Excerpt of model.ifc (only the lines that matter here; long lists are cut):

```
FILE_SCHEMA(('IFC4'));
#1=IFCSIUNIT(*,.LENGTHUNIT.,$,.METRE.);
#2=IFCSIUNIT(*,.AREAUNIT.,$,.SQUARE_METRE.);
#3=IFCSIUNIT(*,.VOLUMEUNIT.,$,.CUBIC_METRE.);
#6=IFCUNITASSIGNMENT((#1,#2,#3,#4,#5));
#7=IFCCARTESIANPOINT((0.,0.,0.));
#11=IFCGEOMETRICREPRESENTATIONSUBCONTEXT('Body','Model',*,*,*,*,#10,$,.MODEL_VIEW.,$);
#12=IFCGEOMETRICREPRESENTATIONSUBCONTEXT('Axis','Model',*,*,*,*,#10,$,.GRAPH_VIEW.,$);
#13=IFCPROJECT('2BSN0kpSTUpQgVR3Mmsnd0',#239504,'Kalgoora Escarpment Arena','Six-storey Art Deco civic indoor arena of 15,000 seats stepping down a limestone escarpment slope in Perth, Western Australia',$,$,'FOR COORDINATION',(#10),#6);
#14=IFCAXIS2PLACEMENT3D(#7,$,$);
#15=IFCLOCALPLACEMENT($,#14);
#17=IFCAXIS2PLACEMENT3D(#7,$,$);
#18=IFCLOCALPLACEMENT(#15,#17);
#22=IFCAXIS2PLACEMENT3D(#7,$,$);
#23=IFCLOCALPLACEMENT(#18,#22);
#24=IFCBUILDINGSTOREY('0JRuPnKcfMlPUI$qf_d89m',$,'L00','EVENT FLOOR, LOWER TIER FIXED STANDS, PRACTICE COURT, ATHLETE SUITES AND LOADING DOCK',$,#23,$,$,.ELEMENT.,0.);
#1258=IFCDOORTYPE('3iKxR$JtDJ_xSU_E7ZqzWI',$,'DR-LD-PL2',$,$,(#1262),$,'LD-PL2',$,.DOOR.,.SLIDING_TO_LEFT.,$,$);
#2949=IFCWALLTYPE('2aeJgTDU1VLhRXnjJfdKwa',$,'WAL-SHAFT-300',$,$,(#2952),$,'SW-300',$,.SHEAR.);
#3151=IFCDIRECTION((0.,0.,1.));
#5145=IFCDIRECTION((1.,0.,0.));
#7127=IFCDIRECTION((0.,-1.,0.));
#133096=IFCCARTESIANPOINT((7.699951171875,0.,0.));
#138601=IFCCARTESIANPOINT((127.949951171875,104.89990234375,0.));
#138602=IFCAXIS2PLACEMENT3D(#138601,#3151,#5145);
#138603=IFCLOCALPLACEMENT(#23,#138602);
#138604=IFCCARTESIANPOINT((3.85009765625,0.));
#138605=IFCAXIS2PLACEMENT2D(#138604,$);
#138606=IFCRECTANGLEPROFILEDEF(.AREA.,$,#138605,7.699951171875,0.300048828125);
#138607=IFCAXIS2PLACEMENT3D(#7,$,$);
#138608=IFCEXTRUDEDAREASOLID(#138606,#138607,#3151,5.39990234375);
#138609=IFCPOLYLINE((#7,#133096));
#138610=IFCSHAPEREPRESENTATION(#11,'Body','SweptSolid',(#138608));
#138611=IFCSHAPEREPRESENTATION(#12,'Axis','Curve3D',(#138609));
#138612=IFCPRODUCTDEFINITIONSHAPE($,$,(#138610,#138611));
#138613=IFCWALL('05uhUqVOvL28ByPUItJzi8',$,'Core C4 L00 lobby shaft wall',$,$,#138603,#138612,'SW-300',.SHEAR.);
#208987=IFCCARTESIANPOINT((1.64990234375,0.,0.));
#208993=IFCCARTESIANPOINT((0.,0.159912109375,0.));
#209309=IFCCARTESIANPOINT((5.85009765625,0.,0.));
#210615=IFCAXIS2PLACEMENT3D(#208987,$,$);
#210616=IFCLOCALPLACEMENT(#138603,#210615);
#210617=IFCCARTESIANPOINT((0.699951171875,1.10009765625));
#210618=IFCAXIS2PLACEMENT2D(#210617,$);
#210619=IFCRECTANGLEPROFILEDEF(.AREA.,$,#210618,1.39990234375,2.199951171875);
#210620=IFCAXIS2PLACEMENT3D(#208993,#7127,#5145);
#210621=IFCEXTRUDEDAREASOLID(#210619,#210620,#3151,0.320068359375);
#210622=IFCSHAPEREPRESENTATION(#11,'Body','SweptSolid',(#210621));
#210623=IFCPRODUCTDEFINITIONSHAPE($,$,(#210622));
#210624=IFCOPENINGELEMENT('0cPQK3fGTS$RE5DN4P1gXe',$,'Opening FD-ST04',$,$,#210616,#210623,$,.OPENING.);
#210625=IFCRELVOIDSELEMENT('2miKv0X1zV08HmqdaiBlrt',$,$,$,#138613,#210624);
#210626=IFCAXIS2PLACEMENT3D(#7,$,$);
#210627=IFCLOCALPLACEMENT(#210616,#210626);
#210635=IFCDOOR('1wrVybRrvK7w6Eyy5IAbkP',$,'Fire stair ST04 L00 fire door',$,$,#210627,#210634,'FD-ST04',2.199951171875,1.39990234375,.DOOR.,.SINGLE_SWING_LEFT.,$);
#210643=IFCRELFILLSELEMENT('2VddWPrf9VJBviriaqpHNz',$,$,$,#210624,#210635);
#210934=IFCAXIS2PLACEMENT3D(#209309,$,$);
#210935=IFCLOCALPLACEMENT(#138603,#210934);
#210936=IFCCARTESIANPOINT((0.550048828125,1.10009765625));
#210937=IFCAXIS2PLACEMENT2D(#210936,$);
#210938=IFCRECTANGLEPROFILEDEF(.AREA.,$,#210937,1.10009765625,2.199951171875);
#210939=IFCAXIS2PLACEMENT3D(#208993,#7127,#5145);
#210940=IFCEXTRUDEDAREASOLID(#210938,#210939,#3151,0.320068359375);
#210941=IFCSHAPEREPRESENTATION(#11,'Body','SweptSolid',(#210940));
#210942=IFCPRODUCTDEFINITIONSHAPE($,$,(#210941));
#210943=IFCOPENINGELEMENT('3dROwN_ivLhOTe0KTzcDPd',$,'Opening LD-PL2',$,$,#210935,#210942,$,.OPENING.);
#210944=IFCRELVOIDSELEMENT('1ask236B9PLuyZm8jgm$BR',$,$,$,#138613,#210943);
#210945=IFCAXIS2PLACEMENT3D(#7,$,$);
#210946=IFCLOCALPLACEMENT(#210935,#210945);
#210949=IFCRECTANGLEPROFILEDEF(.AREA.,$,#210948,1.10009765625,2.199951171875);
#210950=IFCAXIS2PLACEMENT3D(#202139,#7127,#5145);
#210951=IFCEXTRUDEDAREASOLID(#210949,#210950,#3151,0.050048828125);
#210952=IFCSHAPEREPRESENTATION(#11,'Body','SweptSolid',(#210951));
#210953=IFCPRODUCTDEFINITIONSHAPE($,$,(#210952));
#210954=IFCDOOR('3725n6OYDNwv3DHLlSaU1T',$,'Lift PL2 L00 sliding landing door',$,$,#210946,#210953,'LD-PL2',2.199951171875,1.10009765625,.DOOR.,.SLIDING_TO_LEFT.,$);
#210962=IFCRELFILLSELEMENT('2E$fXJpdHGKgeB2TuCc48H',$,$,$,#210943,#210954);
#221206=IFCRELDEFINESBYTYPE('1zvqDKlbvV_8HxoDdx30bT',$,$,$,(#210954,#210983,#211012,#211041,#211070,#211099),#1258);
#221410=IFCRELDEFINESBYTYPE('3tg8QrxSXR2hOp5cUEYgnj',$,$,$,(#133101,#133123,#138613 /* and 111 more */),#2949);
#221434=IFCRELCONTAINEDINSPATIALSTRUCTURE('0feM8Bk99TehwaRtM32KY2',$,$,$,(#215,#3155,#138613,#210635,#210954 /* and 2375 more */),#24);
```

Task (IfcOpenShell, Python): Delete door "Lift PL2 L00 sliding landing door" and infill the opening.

```python
import ifcopenshell
import ifcopenshell.api.feature
import ifcopenshell.api.root
import ifcopenshell.geom
import ifcopenshell.util.shape

model = ifcopenshell.open("model.ifc")
settings = ifcopenshell.geom.settings()


def volume(element):
    """Net volume in cubic metres, openings subtracted."""
    shape = ifcopenshell.geom.create_shape(settings, element)
    return ifcopenshell.util.shape.get_volume(shape.geometry)


door = model.by_id(210954)
opening = door.FillsVoids[0].RelatingOpeningElement
wall = opening.VoidsElements[0].RelatingBuildingElement
before = volume(wall)

ifcopenshell.api.root.remove_product(model, product=door)
ifcopenshell.api.feature.remove_feature(model, feature=opening)

after = volume(wall)

print(f"wall volume {before:.3f} -> {after:.3f} m3")

model.write("model_edited.ifc")
```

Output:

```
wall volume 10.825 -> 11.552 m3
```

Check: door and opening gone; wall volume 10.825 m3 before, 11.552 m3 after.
